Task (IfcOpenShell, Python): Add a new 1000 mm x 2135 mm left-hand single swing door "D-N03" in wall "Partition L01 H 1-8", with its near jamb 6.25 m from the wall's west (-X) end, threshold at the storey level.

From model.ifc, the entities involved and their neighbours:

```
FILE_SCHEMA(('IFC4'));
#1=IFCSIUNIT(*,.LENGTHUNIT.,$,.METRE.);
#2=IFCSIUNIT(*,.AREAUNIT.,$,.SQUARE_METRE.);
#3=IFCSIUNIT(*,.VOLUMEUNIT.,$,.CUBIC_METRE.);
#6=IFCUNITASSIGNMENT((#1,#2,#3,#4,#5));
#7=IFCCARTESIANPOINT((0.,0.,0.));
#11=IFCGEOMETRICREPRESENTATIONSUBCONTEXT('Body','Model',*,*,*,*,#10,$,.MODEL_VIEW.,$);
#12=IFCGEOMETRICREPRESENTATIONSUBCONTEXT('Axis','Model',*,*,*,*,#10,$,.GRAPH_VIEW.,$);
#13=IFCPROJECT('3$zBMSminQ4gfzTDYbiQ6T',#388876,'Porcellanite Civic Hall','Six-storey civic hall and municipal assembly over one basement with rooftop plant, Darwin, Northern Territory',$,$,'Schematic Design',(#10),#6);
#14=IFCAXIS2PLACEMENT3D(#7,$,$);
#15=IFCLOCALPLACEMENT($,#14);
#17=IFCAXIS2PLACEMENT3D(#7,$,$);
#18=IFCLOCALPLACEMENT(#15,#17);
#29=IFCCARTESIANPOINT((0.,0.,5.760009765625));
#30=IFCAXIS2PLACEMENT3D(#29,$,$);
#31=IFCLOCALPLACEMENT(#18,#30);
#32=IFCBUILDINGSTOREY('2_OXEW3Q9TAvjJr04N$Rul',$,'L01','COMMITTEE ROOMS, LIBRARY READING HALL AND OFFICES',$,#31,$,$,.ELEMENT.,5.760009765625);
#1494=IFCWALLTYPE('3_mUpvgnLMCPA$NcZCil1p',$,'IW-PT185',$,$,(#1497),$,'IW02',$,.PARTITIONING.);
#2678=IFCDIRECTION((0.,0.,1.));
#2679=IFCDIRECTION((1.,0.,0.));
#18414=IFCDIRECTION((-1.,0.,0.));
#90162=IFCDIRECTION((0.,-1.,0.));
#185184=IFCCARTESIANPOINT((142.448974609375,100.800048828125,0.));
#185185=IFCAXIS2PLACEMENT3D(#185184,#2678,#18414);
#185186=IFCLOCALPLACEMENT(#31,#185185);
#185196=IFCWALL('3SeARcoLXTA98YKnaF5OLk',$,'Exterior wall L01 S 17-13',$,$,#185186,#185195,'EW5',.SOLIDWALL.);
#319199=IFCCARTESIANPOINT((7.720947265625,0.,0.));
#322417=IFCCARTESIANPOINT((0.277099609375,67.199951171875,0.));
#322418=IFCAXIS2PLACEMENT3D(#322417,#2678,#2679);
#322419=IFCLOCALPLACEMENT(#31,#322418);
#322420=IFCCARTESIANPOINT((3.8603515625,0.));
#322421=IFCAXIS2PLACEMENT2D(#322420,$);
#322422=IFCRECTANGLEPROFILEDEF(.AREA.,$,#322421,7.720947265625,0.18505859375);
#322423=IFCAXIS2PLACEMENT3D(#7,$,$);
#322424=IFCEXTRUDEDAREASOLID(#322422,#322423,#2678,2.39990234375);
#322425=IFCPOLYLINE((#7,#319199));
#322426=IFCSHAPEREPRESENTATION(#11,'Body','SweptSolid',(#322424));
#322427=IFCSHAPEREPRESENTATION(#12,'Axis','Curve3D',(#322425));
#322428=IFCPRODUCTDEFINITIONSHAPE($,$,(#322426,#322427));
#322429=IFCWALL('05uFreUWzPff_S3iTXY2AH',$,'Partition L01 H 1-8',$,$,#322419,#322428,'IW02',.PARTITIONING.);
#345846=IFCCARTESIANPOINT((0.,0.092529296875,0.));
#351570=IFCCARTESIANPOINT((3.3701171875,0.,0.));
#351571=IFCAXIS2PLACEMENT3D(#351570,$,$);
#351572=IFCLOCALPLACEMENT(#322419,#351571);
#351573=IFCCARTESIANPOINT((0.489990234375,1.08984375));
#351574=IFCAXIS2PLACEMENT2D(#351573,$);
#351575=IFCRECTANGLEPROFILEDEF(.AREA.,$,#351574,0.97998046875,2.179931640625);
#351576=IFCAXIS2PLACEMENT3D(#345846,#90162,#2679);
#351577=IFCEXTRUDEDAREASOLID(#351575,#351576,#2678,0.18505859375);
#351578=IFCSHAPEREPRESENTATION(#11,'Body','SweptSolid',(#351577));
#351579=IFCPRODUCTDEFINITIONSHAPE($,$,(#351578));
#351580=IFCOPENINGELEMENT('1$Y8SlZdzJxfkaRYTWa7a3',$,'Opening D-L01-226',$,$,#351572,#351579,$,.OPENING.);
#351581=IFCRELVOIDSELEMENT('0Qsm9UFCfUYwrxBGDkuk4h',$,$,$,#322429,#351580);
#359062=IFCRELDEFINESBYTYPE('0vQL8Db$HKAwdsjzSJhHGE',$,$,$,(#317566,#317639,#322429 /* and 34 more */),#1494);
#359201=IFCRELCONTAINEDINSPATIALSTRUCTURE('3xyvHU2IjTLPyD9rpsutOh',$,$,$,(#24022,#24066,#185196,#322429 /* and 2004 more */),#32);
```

```python
import numpy as np
import ifcopenshell
import ifcopenshell.api.feature
import ifcopenshell.api.geometry
import ifcopenshell.api.root
import ifcopenshell.api.spatial
import ifcopenshell.geom
import ifcopenshell.util.element
import ifcopenshell.util.placement
import ifcopenshell.util.representation
import ifcopenshell.util.shape
import ifcopenshell.util.unit

model = ifcopenshell.open("model.ifc")
unit_scale = ifcopenshell.util.unit.calculate_unit_scale(model)
settings = ifcopenshell.geom.settings()


def volume(element):
    """Net volume in cubic metres, openings subtracted."""
    shape = ifcopenshell.geom.create_shape(settings, element)
    return ifcopenshell.util.shape.get_volume(shape.geometry)


wall = model.by_guid("05uFreUWzPff_S3iTXY2AH")
storey = ifcopenshell.util.element.get_container(wall, ifc_class="IfcBuildingStorey")
context = ifcopenshell.util.representation.get_context(model, "Model", "Body", "MODEL_VIEW")
before = volume(wall)

width, height, from_end, sill = 1, 2.135, 6.25, 0.0  # metres

# The wall runs along its own X axis, and the end named is its -X end.
wall_shape = ifcopenshell.geom.create_shape(settings, wall)
x, y, z = ifcopenshell.util.shape.get_vertices(wall_shape.geometry).T
start = x.min() + from_end
face, thickness = float(y.min()), float(y.max() - y.min())
wall_matrix = ifcopenshell.util.placement.get_local_placement(wall.ObjectPlacement)
level = ifcopenshell.util.placement.get_local_placement(storey.ObjectPlacement)[2, 3]


def in_wall(x, y):
    """Placement at x, y metres in the wall's axes, at sill height."""
    matrix = wall_matrix.copy()
    matrix[:, 3] = wall_matrix @ np.array([x / unit_scale, y / unit_scale, 0.0, 1.0])
    matrix[2, 3] = level + sill / unit_scale
    return matrix


# Opening: a box that overshoots both wall faces by 50 mm.
opening = ifcopenshell.api.root.create_entity(model, ifc_class="IfcOpeningElement", predefined_type="OPENING")
box = ifcopenshell.api.geometry.add_wall_representation(
    model, context=context, length=width, height=height, thickness=thickness + 0.1
)
ifcopenshell.api.geometry.assign_representation(model, product=opening, representation=box)
ifcopenshell.api.geometry.edit_object_placement(model, product=opening, matrix=in_wall(start, face - 0.05), is_si=False)
ifcopenshell.api.feature.add_feature(model, feature=opening, element=wall)

door = ifcopenshell.api.root.create_entity(model, ifc_class="IfcDoor", name="D-N03", predefined_type="DOOR")
door.OverallWidth, door.OverallHeight = width / unit_scale, height / unit_scale
door.OperationType = "SINGLE_SWING_LEFT"
body = ifcopenshell.api.geometry.add_door_representation(
    model,
    context=context,
    overall_width=door.OverallWidth,
    overall_height=door.OverallHeight,
    operation_type="SINGLE_SWING_LEFT",
    lining_properties={"LiningDepth": thickness / unit_scale, "ThresholdDepth": thickness / unit_scale},
)
ifcopenshell.api.geometry.assign_representation(model, product=door, representation=body)
ifcopenshell.api.spatial.assign_container(model, products=[door], relating_structure=storey)
ifcopenshell.api.feature.add_filling(model, opening=opening, element=door)

# The lining spans the wall, so the door starts at the wall face.
ifcopenshell.api.geometry.edit_object_placement(model, product=door, matrix=in_wall(start, face), is_si=False)

after = volume(wall)

print(f"wall volume {before:.3f} -> {after:.3f} m3")

model.write("model_updated.ifc")
```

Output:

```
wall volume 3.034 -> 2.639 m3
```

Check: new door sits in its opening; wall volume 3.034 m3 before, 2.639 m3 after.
